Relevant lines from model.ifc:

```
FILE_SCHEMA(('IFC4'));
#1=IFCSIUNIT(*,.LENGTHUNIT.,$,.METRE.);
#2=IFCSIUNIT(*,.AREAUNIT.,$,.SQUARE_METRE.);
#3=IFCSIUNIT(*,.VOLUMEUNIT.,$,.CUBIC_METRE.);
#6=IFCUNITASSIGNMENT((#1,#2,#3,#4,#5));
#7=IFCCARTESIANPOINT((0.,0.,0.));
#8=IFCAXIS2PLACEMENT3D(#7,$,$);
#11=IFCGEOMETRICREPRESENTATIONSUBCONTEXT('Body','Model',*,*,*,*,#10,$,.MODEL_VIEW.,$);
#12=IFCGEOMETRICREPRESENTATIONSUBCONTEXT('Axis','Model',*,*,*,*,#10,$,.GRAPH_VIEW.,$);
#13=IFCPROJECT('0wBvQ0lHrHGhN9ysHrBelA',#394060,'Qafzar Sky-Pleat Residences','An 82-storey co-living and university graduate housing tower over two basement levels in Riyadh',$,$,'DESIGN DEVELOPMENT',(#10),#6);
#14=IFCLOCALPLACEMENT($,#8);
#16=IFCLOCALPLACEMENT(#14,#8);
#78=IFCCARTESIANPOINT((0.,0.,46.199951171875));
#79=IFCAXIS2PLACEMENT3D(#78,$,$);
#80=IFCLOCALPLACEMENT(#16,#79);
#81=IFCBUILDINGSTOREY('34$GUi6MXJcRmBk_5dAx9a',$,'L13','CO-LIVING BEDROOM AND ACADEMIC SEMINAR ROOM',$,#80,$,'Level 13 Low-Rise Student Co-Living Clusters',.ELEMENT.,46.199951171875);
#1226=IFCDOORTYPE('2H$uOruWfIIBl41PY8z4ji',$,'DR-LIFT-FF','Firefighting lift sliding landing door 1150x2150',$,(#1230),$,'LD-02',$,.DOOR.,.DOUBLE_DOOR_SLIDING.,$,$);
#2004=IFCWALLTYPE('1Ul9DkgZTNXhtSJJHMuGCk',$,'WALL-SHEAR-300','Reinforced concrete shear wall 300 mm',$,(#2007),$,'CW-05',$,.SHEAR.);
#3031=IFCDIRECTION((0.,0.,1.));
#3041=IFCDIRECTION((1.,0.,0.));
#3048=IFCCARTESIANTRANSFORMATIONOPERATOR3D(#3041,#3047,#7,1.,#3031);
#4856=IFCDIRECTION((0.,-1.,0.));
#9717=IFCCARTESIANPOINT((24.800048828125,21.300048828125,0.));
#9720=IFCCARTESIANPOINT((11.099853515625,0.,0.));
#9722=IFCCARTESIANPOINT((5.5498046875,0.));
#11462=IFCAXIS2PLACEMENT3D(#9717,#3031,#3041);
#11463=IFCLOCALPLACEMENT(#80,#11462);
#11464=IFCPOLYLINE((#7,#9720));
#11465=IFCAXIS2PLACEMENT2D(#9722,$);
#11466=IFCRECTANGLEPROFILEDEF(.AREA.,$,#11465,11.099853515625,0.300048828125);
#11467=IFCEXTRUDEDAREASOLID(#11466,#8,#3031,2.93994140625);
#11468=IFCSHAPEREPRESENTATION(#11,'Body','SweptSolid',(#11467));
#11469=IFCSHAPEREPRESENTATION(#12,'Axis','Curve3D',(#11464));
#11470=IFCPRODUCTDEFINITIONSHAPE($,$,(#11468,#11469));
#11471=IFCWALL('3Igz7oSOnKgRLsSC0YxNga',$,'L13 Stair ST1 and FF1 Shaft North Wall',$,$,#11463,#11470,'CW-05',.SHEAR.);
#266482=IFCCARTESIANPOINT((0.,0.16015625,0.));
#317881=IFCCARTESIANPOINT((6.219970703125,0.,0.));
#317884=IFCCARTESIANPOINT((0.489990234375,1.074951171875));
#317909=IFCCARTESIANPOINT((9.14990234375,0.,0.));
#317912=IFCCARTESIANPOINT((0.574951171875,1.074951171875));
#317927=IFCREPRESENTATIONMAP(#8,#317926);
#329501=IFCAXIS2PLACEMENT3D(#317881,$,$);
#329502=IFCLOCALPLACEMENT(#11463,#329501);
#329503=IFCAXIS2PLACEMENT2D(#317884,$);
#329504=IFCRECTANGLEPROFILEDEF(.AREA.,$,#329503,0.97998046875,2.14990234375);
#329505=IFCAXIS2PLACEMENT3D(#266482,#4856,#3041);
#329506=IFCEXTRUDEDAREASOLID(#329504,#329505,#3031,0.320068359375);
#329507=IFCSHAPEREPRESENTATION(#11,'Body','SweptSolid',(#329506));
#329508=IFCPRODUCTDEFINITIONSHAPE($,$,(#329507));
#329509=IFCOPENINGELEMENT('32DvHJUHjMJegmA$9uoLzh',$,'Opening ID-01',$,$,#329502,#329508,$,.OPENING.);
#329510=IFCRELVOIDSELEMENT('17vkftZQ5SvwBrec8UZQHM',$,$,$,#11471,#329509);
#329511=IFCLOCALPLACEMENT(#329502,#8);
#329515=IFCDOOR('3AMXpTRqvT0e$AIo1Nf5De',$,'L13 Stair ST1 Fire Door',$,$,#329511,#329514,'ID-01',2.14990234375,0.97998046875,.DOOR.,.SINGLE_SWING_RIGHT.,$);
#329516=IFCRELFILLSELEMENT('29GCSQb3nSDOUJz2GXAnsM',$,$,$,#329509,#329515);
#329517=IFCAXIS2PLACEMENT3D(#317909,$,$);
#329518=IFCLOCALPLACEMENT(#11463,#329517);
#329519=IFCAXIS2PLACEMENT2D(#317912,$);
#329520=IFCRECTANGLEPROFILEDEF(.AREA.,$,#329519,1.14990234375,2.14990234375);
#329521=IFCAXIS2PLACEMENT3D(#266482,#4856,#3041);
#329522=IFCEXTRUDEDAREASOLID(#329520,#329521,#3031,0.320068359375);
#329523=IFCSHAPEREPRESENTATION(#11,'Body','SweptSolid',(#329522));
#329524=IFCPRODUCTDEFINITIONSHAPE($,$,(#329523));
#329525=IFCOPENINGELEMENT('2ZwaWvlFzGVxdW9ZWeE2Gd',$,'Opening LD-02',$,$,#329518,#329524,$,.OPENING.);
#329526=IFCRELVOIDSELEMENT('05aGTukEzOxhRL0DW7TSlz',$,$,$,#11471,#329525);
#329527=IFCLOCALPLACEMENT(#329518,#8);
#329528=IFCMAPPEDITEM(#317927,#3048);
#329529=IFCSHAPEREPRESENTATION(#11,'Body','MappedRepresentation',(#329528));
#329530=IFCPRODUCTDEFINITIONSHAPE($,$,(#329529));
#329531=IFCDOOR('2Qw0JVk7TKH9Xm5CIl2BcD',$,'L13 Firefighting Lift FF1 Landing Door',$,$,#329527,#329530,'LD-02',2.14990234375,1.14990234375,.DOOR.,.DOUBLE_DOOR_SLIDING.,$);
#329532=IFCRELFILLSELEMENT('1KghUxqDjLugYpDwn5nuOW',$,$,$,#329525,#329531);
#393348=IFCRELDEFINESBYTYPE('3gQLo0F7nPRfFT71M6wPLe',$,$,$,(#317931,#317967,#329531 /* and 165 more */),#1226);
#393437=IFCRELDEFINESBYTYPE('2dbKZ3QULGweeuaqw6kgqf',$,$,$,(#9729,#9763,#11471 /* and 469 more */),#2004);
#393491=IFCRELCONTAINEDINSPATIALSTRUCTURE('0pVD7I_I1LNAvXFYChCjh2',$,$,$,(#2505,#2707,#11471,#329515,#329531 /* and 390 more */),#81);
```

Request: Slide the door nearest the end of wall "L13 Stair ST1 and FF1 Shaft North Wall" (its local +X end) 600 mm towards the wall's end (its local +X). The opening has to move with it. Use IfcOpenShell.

```python
import ifcopenshell
import ifcopenshell.api.geometry
import ifcopenshell.util.placement
import ifcopenshell.util.unit

model = ifcopenshell.open("model.ifc")
unit_scale = ifcopenshell.util.unit.calculate_unit_scale(model)

door = model.by_guid("2Qw0JVk7TKH9Xm5CIl2BcD")
opening = door.FillsVoids[0].RelatingOpeningElement
wall = opening.VoidsElements[0].RelatingBuildingElement

wall_matrix = ifcopenshell.util.placement.get_local_placement(wall.ObjectPlacement)
shift = wall_matrix[:3, 0] * 0.6 / unit_scale
before = ifcopenshell.util.placement.get_local_placement(door.ObjectPlacement)[:3, 3].copy()

# The door is placed relative to its opening, so it follows when the opening moves.
matrix = ifcopenshell.util.placement.get_local_placement(opening.ObjectPlacement)
matrix[:3, 3] += shift
ifcopenshell.api.geometry.edit_object_placement(
    model, product=opening, matrix=matrix, is_si=False, should_transform_children=True
)

after = ifcopenshell.util.placement.get_local_placement(door.ObjectPlacement)[:3, 3]
print("door moved by", (after - before).round(3) + 0.0)

model.write("model_v2.ifc")
```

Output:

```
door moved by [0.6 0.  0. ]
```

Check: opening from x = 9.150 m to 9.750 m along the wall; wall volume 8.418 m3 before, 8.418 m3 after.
